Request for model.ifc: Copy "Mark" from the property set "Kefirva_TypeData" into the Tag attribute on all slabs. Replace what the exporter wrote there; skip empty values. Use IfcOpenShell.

First a look at what the model holds.

```python
import ifcopenshell
import ifcopenshell.util.element

model = ifcopenshell.open("model.ifc")
print(model.schema)
slabs = model.by_type("IfcSlab")
print(len(slabs), "slabs")
for e in slabs[:8]:
    source = ifcopenshell.util.element.get_pset(e, "Kefirva_TypeData", "Mark")
    target = e.Tag
    print(e.id(), repr(source), repr(target), sep=" | ")
```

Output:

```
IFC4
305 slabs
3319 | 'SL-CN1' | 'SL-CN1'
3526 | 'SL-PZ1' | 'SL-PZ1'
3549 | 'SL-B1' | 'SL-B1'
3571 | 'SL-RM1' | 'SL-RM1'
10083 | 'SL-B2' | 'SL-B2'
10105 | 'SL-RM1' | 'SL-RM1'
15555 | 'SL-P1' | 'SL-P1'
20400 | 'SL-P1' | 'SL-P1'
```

```python
import ifcopenshell
import ifcopenshell.util.element

model = ifcopenshell.open("model.ifc")

count = 0
for e in model.by_type("IfcSlab"):
    value = ifcopenshell.util.element.get_pset(e, "Kefirva_TypeData", "Mark")
    current = e.Tag
    if not value or not value.strip() or current == value:
        continue
    e.Tag = value
    count += 1

print(count, "slabs updated")

model.write("model_updated.ifc")
```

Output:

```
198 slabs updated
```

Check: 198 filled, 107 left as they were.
